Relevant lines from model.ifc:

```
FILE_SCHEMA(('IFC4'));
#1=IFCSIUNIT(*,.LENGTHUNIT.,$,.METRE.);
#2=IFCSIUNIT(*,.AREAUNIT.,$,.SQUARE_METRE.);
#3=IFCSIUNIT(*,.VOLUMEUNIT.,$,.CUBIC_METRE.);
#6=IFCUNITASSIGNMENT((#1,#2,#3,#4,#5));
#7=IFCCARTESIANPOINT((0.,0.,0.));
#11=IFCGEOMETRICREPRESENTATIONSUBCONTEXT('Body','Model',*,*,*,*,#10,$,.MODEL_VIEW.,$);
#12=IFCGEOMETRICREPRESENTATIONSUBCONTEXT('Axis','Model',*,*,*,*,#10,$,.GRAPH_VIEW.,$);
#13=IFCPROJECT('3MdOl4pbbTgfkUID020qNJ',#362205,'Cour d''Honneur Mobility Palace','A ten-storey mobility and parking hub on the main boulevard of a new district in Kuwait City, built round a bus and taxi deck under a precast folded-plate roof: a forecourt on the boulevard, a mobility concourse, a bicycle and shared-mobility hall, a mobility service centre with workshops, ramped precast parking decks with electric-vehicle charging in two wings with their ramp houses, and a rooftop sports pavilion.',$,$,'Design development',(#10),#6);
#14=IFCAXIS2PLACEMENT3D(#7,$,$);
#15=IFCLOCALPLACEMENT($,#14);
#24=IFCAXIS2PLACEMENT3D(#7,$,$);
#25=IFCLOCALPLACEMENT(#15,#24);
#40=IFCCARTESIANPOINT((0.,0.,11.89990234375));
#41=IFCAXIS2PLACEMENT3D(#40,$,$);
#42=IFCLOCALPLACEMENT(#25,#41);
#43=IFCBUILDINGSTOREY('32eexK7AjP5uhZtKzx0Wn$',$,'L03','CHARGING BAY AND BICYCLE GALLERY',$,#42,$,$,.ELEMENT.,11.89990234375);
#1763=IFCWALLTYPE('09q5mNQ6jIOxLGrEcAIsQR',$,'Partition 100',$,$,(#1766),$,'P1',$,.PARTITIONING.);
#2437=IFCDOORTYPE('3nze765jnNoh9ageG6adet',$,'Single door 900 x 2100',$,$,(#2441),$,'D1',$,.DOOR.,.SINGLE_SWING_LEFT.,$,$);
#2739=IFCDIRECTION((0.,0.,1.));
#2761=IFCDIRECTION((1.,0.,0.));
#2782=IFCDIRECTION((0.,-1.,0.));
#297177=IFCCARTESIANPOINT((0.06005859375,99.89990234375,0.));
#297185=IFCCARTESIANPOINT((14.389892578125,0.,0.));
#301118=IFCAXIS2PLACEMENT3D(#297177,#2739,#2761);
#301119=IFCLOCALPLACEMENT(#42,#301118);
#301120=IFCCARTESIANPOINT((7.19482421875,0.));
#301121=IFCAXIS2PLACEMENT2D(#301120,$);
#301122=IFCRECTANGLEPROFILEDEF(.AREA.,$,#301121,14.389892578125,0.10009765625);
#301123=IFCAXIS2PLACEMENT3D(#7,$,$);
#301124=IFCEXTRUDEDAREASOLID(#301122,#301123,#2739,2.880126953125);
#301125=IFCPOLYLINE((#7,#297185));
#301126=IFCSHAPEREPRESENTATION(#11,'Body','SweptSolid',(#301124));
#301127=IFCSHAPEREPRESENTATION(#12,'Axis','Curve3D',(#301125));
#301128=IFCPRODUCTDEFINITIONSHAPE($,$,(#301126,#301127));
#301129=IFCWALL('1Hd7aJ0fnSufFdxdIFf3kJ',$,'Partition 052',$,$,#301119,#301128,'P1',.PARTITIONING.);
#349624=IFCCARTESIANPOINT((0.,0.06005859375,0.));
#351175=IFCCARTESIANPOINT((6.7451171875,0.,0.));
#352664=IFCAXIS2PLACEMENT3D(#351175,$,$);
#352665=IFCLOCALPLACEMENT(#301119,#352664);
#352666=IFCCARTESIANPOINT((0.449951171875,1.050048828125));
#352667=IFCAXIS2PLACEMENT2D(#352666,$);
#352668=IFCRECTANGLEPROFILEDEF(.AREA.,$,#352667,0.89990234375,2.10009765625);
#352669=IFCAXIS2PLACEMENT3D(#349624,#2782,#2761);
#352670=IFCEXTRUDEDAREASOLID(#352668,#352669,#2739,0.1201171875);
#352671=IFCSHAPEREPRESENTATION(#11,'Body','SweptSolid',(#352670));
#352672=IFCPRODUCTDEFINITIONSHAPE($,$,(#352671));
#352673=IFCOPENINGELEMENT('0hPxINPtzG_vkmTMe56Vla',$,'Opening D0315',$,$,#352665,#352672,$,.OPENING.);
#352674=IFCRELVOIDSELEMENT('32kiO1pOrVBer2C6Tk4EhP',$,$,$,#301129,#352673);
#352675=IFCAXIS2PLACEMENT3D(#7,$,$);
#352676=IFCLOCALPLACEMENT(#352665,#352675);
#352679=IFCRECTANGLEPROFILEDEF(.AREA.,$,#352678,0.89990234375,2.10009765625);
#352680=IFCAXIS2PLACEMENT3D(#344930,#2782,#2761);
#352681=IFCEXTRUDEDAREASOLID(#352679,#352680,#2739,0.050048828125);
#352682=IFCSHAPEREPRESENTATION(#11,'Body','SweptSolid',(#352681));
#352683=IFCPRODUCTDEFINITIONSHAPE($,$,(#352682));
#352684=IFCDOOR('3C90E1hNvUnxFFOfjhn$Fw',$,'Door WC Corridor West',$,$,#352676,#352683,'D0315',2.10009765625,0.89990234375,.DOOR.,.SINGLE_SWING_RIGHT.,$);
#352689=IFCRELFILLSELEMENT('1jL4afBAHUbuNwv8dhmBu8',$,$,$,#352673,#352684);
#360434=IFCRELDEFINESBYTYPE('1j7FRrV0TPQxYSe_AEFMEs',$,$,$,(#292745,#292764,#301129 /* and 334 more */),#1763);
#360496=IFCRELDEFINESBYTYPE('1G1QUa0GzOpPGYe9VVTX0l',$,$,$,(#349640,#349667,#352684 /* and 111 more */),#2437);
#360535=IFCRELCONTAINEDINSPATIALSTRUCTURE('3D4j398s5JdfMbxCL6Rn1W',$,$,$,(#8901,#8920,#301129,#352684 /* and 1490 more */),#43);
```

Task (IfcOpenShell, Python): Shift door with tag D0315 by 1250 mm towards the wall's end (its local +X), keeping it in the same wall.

```python
import ifcopenshell
import ifcopenshell.api.geometry
import ifcopenshell.util.placement
import ifcopenshell.util.unit

model = ifcopenshell.open("model.ifc")
unit_scale = ifcopenshell.util.unit.calculate_unit_scale(model)

door = model.by_guid("3C90E1hNvUnxFFOfjhn$Fw")
opening = door.FillsVoids[0].RelatingOpeningElement
wall = opening.VoidsElements[0].RelatingBuildingElement

wall_matrix = ifcopenshell.util.placement.get_local_placement(wall.ObjectPlacement)
shift = wall_matrix[:3, 0] * 1.25 / unit_scale
before = ifcopenshell.util.placement.get_local_placement(door.ObjectPlacement)[:3, 3].copy()

# The door is placed relative to its opening, so it follows when the opening moves.
matrix = ifcopenshell.util.placement.get_local_placement(opening.ObjectPlacement)
matrix[:3, 3] += shift
ifcopenshell.api.geometry.edit_object_placement(
    model, product=opening, matrix=matrix, is_si=False, should_transform_children=True
)

after = ifcopenshell.util.placement.get_local_placement(door.ObjectPlacement)[:3, 3]
print("door moved by", (after - before).round(3) + 0.0)

model.write("model_updated.ifc")
```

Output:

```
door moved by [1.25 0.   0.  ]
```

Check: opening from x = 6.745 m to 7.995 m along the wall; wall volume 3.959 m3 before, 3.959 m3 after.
